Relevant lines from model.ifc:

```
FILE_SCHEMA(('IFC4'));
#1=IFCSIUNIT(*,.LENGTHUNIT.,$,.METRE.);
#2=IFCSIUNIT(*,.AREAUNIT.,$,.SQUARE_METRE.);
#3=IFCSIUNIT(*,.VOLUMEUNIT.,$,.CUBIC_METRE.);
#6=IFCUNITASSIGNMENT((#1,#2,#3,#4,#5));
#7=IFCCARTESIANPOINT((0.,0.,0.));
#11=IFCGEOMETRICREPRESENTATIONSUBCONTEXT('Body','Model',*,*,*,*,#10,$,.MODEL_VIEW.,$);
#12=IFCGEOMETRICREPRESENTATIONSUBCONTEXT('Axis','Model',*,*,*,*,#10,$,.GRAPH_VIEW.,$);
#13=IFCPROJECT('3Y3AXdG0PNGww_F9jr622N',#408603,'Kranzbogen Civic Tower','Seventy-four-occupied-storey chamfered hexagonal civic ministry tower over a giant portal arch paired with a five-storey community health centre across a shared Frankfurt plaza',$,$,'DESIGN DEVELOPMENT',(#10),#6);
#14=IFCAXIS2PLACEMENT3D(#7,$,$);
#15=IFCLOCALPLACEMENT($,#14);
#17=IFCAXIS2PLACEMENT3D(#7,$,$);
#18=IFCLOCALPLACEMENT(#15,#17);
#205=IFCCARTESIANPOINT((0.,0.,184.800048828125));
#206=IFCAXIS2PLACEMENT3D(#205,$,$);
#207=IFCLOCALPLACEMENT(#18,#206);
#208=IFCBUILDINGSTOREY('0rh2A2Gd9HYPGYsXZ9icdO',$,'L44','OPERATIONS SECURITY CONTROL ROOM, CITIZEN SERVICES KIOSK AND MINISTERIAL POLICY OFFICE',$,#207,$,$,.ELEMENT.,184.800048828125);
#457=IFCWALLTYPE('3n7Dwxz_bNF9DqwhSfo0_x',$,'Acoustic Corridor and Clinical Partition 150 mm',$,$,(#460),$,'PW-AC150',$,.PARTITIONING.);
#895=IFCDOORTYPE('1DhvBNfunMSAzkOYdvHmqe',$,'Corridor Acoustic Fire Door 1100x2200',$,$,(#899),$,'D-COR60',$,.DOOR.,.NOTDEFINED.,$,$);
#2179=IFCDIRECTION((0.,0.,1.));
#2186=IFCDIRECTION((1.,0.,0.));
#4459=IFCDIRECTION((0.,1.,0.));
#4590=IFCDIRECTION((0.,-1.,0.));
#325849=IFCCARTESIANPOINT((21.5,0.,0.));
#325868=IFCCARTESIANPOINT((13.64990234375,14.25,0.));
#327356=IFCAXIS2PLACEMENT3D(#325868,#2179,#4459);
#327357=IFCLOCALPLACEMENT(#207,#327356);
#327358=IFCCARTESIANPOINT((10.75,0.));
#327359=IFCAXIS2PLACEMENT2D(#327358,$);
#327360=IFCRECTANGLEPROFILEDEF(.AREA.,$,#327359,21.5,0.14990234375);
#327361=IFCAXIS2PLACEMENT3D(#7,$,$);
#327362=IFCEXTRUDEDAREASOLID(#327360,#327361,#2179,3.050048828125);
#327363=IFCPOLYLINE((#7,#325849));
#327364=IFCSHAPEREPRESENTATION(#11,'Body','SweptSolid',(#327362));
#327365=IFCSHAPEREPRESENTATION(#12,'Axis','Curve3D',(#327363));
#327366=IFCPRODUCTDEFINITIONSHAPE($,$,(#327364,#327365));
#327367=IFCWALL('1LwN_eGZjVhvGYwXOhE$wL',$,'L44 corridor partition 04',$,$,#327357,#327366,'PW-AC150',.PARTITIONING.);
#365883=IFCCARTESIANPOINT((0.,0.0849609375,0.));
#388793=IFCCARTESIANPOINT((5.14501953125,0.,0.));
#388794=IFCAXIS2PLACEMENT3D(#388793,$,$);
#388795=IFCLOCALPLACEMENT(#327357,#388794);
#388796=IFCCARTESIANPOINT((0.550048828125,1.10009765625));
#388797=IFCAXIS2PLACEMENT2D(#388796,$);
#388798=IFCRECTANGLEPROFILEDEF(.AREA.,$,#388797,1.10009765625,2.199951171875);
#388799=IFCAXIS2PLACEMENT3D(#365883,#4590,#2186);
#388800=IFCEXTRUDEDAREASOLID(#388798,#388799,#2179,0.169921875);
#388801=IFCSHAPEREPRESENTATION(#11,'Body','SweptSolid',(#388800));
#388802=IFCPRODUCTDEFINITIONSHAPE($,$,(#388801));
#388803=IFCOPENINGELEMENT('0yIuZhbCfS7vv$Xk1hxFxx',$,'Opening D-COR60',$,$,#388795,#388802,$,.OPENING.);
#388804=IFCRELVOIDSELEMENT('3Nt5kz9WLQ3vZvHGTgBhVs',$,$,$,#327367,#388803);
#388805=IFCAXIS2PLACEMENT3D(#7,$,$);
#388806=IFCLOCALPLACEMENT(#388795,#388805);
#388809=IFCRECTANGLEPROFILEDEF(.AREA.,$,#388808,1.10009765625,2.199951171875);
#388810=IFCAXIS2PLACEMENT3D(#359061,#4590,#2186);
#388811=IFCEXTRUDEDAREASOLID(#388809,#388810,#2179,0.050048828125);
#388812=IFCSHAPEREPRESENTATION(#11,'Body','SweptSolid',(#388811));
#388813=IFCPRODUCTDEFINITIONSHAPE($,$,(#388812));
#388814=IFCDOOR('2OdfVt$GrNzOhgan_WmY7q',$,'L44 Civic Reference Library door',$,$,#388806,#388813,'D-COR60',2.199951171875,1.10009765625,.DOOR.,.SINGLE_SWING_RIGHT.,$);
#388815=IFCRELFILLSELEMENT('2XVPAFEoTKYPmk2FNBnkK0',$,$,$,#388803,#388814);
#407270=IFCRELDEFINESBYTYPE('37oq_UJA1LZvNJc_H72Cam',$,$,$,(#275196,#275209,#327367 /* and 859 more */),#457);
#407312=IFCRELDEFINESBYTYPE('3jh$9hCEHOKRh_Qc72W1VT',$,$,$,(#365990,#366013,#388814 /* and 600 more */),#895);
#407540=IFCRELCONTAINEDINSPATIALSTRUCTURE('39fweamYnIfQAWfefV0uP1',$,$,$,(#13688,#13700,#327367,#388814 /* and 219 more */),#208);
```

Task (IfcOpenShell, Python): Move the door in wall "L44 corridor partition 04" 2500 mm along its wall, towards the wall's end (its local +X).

```python
import ifcopenshell
import ifcopenshell.api.geometry
import ifcopenshell.util.placement
import ifcopenshell.util.unit

model = ifcopenshell.open("model.ifc")
unit_scale = ifcopenshell.util.unit.calculate_unit_scale(model)

door = model.by_guid("2OdfVt$GrNzOhgan_WmY7q")
opening = door.FillsVoids[0].RelatingOpeningElement
wall = opening.VoidsElements[0].RelatingBuildingElement

wall_matrix = ifcopenshell.util.placement.get_local_placement(wall.ObjectPlacement)
shift = wall_matrix[:3, 0] * 2.5 / unit_scale
before = ifcopenshell.util.placement.get_local_placement(door.ObjectPlacement)[:3, 3].copy()

# The door is placed relative to its opening, so it follows when the opening moves.
matrix = ifcopenshell.util.placement.get_local_placement(opening.ObjectPlacement)
matrix[:3, 3] += shift
ifcopenshell.api.geometry.edit_object_placement(
    model, product=opening, matrix=matrix, is_si=False, should_transform_children=True
)

after = ifcopenshell.util.placement.get_local_placement(door.ObjectPlacement)[:3, 3]
print("door moved by", (after - before).round(3) + 0.0)

model.write("model-out.ifc")
```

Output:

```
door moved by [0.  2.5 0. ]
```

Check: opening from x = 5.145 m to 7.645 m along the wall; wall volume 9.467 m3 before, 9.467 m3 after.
